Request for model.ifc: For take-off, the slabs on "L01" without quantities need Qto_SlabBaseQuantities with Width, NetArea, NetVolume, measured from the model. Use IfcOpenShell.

First a look at what the model holds.

```python
import ifcopenshell
import ifcopenshell.util.element
import ifcopenshell.util.unit

model = ifcopenshell.open("model.ifc")
print(model.schema)
for unit_type in ("LENGTHUNIT", "AREAUNIT", "VOLUMEUNIT"):
    print(unit_type, ifcopenshell.util.unit.calculate_unit_scale(model, unit_type))
storey = next(s for s in model.by_type("IfcBuildingStorey") if s.Name == "L01")
slabs = [e for e in ifcopenshell.util.element.get_decomposition(storey) if e.is_a("IfcSlab")]
for e in sorted(slabs, key=lambda e: e.id()):
    print(e.id(), e.is_a(), e.Name, list(ifcopenshell.util.element.get_psets(e, qtos_only=True)), sep=" | ")
```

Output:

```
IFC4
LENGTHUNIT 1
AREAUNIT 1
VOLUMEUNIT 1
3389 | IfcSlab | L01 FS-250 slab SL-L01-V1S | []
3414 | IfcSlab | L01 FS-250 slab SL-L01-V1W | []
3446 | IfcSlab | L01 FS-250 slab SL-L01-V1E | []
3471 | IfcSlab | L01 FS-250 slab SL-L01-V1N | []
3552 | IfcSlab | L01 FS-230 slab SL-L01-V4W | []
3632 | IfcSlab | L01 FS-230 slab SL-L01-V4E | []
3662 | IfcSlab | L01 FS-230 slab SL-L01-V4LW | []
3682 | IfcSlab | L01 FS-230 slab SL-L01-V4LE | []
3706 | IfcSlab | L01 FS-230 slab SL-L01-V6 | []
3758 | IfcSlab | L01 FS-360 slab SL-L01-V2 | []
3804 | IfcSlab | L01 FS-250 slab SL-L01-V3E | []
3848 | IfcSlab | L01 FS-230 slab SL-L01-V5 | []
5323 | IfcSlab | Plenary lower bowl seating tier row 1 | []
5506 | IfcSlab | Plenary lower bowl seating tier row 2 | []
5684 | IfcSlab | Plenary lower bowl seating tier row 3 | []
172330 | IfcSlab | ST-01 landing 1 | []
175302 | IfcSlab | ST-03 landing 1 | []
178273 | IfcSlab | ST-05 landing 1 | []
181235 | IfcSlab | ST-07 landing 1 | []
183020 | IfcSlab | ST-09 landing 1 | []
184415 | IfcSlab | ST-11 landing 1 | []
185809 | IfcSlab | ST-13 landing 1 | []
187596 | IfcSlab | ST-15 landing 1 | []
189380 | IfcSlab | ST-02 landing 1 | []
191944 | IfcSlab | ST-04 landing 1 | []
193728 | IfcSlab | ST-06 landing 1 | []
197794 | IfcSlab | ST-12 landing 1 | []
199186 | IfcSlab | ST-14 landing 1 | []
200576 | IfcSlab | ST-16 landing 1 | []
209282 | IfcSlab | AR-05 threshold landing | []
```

```python
import ifcopenshell
import ifcopenshell.api.pset
import ifcopenshell.geom
import ifcopenshell.util.element
import ifcopenshell.util.shape
import ifcopenshell.util.unit

model = ifcopenshell.open("model.ifc")
unit_scale = ifcopenshell.util.unit.calculate_unit_scale(model)
area_scale = ifcopenshell.util.unit.calculate_unit_scale(model, "AREAUNIT")
volume_scale = ifcopenshell.util.unit.calculate_unit_scale(model, "VOLUMEUNIT")
settings = ifcopenshell.geom.settings()

storey = next(s for s in model.by_type("IfcBuildingStorey") if s.Name == "L01")
slabs = [e for e in ifcopenshell.util.element.get_decomposition(storey) if e.is_a("IfcSlab")]

for e in sorted(slabs, key=lambda e: e.id()):
    if ifcopenshell.util.element.get_psets(e, qtos_only=True, should_inherit=False):
        continue
    # Geometry comes back in metres, in the element's own axes.
    shape = ifcopenshell.geom.create_shape(settings, e)
    values = {
        "Width": ifcopenshell.util.shape.get_z(shape.geometry) / unit_scale,
        "NetArea": ifcopenshell.util.shape.get_footprint_area(shape.geometry) / area_scale,
        "NetVolume": ifcopenshell.util.shape.get_volume(shape.geometry) / volume_scale,
    }
    qto = ifcopenshell.api.pset.add_qto(model, product=e, name="Qto_SlabBaseQuantities")
    ifcopenshell.api.pset.edit_qto(model, qto=qto, properties=values)
    print(e.id(), {k: round(v, 3) for k, v in values.items()})

model.write("model_v2.ifc")
```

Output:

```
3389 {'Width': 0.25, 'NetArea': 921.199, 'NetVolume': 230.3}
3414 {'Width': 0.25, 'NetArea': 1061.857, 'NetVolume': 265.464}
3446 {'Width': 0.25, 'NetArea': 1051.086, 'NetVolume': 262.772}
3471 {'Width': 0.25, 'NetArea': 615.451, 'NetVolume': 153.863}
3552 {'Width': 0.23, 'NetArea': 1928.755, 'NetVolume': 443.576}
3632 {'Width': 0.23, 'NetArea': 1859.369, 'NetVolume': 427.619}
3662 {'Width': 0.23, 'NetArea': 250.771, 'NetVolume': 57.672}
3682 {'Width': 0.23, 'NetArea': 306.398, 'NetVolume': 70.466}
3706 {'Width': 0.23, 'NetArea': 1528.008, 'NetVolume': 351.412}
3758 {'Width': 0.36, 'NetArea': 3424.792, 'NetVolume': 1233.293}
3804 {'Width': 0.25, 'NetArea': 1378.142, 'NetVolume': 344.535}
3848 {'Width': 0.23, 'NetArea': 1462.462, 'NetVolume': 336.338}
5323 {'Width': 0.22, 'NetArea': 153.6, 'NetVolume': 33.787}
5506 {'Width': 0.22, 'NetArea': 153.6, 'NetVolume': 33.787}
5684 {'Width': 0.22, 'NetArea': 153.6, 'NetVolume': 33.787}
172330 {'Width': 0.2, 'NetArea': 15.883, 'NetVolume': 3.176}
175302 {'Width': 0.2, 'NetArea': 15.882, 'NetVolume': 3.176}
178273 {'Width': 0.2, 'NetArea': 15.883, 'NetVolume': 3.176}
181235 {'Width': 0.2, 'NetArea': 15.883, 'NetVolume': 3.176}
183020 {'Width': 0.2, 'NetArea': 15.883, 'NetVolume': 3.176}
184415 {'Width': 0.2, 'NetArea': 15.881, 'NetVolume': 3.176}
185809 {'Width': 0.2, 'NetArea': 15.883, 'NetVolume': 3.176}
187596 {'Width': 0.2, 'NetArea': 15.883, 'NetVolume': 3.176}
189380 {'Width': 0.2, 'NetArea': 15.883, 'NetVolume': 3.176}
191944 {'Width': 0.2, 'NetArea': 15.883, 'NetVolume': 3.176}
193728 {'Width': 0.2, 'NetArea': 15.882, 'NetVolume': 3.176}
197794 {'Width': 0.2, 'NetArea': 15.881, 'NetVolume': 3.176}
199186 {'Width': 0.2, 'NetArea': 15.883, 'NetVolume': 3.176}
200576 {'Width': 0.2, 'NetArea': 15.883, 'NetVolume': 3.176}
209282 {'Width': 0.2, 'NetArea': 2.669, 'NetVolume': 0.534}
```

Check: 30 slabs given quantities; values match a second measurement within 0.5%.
